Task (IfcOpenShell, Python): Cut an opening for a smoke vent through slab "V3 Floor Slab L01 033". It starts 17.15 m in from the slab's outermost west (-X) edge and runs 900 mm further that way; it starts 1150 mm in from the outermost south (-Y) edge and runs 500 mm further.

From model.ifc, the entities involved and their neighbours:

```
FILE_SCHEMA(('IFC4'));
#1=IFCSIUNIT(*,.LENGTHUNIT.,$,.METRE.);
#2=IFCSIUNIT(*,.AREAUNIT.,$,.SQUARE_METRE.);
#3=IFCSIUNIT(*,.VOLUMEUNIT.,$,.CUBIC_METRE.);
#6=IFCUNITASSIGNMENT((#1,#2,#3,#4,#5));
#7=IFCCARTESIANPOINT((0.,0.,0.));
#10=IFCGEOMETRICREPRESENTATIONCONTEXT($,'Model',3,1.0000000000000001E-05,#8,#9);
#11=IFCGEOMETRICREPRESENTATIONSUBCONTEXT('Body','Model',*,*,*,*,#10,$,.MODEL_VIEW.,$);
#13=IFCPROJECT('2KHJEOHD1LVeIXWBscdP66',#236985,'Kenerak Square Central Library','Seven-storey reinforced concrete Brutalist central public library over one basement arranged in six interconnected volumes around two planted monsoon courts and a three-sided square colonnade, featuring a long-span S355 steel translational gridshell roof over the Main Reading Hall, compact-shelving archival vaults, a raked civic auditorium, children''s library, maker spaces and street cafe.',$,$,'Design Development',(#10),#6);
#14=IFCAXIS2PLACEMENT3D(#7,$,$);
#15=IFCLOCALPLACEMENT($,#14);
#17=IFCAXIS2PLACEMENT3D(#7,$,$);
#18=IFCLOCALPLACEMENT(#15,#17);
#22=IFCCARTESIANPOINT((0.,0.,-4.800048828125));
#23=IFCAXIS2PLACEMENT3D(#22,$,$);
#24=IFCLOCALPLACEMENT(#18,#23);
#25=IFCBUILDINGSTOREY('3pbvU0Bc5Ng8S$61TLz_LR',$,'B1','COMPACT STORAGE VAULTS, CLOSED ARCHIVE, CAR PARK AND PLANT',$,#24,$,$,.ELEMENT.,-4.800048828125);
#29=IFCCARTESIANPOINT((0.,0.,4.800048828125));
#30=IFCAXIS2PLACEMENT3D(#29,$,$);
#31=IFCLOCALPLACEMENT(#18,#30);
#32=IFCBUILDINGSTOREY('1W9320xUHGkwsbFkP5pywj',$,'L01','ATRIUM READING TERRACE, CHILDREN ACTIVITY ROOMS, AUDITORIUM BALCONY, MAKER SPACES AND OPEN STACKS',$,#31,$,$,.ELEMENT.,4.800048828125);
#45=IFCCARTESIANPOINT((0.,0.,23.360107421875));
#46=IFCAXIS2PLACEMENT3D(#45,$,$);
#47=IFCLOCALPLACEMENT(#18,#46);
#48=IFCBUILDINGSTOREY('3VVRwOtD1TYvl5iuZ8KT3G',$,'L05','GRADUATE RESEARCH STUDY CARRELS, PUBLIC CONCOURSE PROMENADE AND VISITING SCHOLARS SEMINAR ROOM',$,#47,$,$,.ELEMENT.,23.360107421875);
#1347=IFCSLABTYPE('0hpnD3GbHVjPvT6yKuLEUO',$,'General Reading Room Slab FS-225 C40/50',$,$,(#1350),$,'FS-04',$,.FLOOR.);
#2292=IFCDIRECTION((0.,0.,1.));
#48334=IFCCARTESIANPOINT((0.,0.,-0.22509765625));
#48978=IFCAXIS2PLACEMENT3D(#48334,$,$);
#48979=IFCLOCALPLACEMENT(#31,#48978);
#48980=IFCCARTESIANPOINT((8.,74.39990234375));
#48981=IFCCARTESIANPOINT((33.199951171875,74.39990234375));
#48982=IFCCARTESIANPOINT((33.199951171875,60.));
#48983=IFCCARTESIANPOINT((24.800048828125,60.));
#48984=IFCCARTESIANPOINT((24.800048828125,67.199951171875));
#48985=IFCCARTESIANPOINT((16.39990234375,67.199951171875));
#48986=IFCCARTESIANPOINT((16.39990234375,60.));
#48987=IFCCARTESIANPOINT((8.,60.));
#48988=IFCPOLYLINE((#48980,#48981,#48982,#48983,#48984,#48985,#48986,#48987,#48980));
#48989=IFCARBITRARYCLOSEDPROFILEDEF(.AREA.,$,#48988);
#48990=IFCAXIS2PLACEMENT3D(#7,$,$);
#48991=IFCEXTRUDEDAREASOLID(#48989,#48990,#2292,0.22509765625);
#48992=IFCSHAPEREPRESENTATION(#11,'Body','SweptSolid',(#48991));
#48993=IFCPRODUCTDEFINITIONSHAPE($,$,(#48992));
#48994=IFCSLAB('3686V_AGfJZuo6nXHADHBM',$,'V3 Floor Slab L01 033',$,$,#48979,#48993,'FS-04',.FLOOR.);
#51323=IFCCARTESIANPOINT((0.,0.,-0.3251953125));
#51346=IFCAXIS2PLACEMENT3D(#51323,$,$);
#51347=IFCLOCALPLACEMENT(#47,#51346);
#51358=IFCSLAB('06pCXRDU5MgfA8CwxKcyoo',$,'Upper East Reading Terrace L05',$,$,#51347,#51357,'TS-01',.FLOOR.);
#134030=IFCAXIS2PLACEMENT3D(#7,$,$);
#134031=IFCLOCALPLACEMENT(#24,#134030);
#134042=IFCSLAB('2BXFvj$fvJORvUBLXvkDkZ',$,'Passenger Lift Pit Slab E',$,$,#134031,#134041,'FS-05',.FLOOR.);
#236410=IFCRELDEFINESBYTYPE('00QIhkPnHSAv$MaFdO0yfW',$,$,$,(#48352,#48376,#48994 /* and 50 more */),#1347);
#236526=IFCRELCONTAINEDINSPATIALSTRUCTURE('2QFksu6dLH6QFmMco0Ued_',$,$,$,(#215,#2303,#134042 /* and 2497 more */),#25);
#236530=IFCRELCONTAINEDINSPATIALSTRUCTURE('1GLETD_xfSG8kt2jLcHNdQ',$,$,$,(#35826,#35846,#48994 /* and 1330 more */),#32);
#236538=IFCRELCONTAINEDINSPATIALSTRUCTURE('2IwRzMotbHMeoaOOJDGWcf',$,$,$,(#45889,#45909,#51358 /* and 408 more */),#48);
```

```python
import numpy as np
import ifcopenshell
import ifcopenshell.api.feature
import ifcopenshell.api.geometry
import ifcopenshell.api.root
import ifcopenshell.geom
import ifcopenshell.util.placement
import ifcopenshell.util.representation
import ifcopenshell.util.shape
import ifcopenshell.util.unit

model = ifcopenshell.open("model.ifc")
unit_scale = ifcopenshell.util.unit.calculate_unit_scale(model)
settings = ifcopenshell.geom.settings()


def volume(element):
    """Net volume in cubic metres, openings subtracted."""
    shape = ifcopenshell.geom.create_shape(settings, element)
    return ifcopenshell.util.shape.get_volume(shape.geometry)


slab = model.by_guid("3686V_AGfJZuo6nXHADHBM")
before = volume(slab)

# Extent in the slab's own axes, in metres. The edges named are its -X and -Y sides.
slab_shape = ifcopenshell.geom.create_shape(settings, slab)
vertices = ifcopenshell.util.shape.get_vertices(slab_shape.geometry)
x_min, y_min, bottom = vertices.min(axis=0)
top = vertices[:, 2].max()

opening = ifcopenshell.api.root.create_entity(model, ifc_class="IfcOpeningElement", name="Smoke vent opening", predefined_type="OPENING")
context = ifcopenshell.util.representation.get_context(model, "Model", "Body", "MODEL_VIEW")
width, depth = 0.9, 0.5
outline = [(0.0, 0.0), (width, 0.0), (width, depth), (0.0, depth), (0.0, 0.0)]
# Overshoot both faces by 50 mm so the cut is clean.
shape = ifcopenshell.api.geometry.add_slab_representation(
    model, context=context, depth=top - bottom + 0.1, polyline=outline
)
ifcopenshell.api.geometry.assign_representation(model, product=opening, representation=shape)

matrix = ifcopenshell.util.placement.get_local_placement(slab.ObjectPlacement)
matrix[:, 3] = matrix @ np.append(np.array([x_min + 17.15, y_min + 1.15, bottom - 0.05]) / unit_scale, 1.0)
ifcopenshell.api.geometry.edit_object_placement(model, product=opening, matrix=matrix, is_si=False)
ifcopenshell.api.feature.add_feature(model, feature=opening, element=slab)

after = volume(slab)

print(f"slab volume {before:.3f} -> {after:.3f} m3")

model.write("model_v2.ifc")
```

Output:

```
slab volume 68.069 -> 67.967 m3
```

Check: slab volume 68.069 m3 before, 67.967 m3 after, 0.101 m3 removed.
